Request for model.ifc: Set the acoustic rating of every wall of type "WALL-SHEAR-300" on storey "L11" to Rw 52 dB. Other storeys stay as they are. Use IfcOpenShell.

First a look at what the model holds.

```python
import ifcopenshell
import ifcopenshell.util.element

model = ifcopenshell.open("model.ifc")
print(model.schema)
storey = next(s for s in model.by_type("IfcBuildingStorey") if s.Name == "L11")
walls = [e for e in ifcopenshell.util.element.get_decomposition(storey) if e.is_a("IfcWall")]
seen = {}
for e in walls:
    element_type = ifcopenshell.util.element.get_type(e)
    key = (element_type.Name if element_type != e and element_type else None, ifcopenshell.util.element.get_pset(e, "Pset_WallCommon", "AcousticRating"))
    seen[key] = seen.get(key, 0) + 1
for (name, value), count in sorted(seen.items(), key=str):
    print(count, "x", name, "|", value)
```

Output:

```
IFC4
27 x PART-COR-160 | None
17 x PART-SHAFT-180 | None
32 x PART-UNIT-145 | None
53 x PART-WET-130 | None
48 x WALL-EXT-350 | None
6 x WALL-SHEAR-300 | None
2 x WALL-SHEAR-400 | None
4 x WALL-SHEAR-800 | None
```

```python
import ifcopenshell
import ifcopenshell.api.pset
import ifcopenshell.util.element

model = ifcopenshell.open("model.ifc")

storey = next(s for s in model.by_type("IfcBuildingStorey") if s.Name == "L11")
walls = [e for e in ifcopenshell.util.element.get_decomposition(storey) if e.is_a("IfcWall")]

count = 0
for e in walls:
    element_type = ifcopenshell.util.element.get_type(e)
    if element_type in (None, e) or element_type.Name != "WALL-SHEAR-300":
        continue
    found = ifcopenshell.util.element.get_pset(e, "Pset_WallCommon", should_inherit=False)
    if found:
        pset = model.by_id(found["id"])
        if len(ifcopenshell.util.element.get_elements_by_pset(pset)) > 1:
            pset = ifcopenshell.api.pset.unshare_pset(model, products=[e], pset=pset)[0]
    else:
        pset = ifcopenshell.api.pset.add_pset(model, product=e, name="Pset_WallCommon")
    ifcopenshell.api.pset.edit_pset(model, pset=pset, properties={"AcousticRating": "Rw 52 dB"})
    count += 1

print(count, "walls updated")

model.write("model_v2.ifc")
```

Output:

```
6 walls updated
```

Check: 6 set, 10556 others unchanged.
